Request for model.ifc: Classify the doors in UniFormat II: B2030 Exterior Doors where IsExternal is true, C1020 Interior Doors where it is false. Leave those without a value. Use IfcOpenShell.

First a look at what the model holds.

```python
import ifcopenshell
import ifcopenshell.util.element

model = ifcopenshell.open("model.ifc")
print(model.schema)
print("classifications:", [c.Name for c in model.by_type("IfcClassification")])
values = [ifcopenshell.util.element.get_pset(e, "Pset_DoorCommon", "IsExternal") for e in model.by_type("IfcDoor")]
for value in (True, False, None):
    print("IsExternal", value, values.count(value))
```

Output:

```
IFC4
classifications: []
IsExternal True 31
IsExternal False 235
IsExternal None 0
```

```python
import ifcopenshell
import ifcopenshell.api.classification
import ifcopenshell.util.element

model = ifcopenshell.open("model.ifc")

system = ifcopenshell.api.classification.add_classification(model, classification="UniFormat II")

doors = model.by_type("IfcDoor")
external = {e: ifcopenshell.util.element.get_pset(e, "Pset_DoorCommon", "IsExternal") for e in doors}
for flag, code, name in ((True, "B2030", "Exterior Doors"), (False, "C1020", "Interior Doors")):
    products = [e for e in doors if external[e] is flag]
    ifcopenshell.api.classification.add_reference(
        model, products=products, classification=system, identification=code, name=name
    )
    print(code, len(products))

model.write("model_edited.ifc")
```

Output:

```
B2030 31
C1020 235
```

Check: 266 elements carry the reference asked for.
